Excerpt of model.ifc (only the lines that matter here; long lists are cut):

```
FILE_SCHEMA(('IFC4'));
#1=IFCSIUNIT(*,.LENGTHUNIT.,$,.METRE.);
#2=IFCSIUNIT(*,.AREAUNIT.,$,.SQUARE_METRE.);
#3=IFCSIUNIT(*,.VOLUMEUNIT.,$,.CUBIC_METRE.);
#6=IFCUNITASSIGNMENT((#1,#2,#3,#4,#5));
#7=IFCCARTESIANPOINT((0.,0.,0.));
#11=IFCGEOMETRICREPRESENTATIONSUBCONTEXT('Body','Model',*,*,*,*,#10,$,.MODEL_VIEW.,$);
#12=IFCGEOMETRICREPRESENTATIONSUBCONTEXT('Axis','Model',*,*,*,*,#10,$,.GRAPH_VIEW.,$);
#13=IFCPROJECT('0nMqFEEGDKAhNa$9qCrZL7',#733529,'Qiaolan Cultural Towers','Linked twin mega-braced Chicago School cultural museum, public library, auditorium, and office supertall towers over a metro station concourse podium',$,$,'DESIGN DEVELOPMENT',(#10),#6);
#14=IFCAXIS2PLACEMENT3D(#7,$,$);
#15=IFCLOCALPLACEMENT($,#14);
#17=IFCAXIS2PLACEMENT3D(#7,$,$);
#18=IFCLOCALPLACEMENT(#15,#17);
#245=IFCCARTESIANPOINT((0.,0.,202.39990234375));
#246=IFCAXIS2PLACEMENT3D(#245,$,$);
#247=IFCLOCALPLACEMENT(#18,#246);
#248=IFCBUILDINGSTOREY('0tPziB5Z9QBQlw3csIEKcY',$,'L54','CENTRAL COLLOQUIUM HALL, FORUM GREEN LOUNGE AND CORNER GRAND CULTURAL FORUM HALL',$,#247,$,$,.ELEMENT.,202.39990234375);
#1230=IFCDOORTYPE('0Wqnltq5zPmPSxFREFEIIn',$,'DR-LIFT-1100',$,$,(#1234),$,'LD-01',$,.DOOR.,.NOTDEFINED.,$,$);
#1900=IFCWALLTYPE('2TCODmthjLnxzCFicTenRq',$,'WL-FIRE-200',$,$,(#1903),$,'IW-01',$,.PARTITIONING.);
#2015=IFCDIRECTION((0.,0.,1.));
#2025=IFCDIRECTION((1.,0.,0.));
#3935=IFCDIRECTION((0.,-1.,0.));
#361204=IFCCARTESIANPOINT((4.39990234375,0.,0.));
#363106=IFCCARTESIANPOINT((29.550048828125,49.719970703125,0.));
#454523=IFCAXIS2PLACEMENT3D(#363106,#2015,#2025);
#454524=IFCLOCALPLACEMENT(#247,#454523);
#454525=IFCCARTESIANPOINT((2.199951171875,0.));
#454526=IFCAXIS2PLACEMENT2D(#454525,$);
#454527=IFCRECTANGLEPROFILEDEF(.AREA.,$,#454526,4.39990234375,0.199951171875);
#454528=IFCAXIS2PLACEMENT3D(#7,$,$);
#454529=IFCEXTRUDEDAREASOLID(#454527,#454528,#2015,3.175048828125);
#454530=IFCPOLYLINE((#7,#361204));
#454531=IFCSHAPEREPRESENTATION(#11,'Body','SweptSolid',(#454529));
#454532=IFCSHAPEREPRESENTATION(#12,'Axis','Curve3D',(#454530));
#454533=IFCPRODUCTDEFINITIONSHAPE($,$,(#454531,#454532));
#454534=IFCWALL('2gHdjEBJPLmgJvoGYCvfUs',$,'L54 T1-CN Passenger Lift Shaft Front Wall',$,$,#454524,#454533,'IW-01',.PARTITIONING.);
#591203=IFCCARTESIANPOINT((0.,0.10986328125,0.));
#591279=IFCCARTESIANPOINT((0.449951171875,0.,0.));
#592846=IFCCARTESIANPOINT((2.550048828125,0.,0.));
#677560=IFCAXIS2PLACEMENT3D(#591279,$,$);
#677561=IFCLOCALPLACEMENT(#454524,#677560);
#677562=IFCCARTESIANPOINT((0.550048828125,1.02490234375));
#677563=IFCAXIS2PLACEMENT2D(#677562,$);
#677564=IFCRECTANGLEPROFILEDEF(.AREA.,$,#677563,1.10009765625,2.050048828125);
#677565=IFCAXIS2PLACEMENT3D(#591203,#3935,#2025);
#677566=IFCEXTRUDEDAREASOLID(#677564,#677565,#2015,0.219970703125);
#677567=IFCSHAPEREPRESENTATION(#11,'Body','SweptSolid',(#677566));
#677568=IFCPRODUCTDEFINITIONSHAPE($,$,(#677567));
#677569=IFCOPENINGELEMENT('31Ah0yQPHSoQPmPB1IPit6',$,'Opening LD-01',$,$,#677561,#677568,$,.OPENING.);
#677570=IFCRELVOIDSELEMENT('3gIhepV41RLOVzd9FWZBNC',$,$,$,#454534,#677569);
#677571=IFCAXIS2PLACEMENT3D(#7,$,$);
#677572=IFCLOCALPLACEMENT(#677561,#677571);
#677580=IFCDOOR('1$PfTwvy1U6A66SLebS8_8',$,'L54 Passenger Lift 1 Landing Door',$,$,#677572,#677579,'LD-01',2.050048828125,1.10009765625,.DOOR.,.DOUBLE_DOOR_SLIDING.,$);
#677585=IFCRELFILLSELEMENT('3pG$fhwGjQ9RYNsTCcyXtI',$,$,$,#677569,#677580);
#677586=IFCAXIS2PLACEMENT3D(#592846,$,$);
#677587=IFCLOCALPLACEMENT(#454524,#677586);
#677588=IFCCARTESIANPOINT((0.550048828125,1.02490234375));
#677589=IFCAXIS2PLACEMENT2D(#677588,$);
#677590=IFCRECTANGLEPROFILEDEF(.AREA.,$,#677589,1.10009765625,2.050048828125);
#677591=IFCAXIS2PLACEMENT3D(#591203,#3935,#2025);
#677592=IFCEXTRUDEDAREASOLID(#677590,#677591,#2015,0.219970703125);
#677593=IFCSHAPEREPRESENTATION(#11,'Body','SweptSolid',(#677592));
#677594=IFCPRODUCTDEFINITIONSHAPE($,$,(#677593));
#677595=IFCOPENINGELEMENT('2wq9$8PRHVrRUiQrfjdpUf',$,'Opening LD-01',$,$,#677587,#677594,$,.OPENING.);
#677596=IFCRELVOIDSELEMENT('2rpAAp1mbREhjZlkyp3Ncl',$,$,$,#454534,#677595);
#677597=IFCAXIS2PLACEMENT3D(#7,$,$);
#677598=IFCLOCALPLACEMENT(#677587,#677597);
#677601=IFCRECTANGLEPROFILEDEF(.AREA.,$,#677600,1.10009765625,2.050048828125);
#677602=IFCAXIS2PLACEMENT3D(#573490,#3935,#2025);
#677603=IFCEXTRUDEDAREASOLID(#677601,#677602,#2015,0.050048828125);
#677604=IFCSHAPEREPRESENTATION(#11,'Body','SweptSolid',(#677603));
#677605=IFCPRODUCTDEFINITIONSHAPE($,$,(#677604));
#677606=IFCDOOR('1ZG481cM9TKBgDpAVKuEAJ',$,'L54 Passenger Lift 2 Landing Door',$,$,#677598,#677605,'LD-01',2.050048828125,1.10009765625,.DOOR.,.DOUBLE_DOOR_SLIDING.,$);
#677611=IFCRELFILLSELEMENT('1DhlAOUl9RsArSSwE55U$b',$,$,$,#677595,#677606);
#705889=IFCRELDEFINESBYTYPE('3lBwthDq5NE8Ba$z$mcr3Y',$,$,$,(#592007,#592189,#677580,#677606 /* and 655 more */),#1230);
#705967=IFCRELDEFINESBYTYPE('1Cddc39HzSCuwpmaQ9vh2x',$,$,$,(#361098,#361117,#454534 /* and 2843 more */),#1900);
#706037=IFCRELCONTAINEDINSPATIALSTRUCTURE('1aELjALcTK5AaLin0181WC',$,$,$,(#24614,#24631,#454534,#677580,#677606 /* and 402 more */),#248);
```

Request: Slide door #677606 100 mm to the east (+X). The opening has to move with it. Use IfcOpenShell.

```python
import ifcopenshell
import ifcopenshell.api.geometry
import ifcopenshell.util.placement

model = ifcopenshell.open("model.ifc")

door = model.by_guid("1ZG481cM9TKBgDpAVKuEAJ")
opening = door.FillsVoids[0].RelatingOpeningElement
wall = opening.VoidsElements[0].RelatingBuildingElement

wall_matrix = ifcopenshell.util.placement.get_local_placement(wall.ObjectPlacement)
shift = wall_matrix[:3, 0] * 0.1
before = ifcopenshell.util.placement.get_local_placement(door.ObjectPlacement)[:3, 3].copy()

# The door is placed relative to its opening, so it follows when the opening moves.
matrix = ifcopenshell.util.placement.get_local_placement(opening.ObjectPlacement)
matrix[:3, 3] += shift
ifcopenshell.api.geometry.edit_object_placement(
    model, product=opening, matrix=matrix, is_si=False, should_transform_children=True
)

after = ifcopenshell.util.placement.get_local_placement(door.ObjectPlacement)[:3, 3]
print("door moved by", (after - before).round(3) + 0.0)

model.write("model-out.ifc")
```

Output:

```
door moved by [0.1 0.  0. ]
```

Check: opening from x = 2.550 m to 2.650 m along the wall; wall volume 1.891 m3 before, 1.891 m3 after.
